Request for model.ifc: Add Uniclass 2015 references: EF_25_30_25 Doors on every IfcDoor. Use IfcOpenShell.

First a look at what the model holds.

```python
import ifcopenshell

model = ifcopenshell.open("model.ifc")
print(model.schema)
print("classifications:", [c.Name for c in model.by_type("IfcClassification")])
for ifc_class in ("IfcDoor", "IfcRoof", "IfcStair", "IfcWall", "IfcWindow"):
    print(ifc_class, len(model.by_type(ifc_class)))
```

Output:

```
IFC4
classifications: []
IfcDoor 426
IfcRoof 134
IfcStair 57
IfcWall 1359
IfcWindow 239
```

```python
import ifcopenshell
import ifcopenshell.api.classification

model = ifcopenshell.open("model.ifc")

system = ifcopenshell.api.classification.add_classification(model, classification="Uniclass 2015")

codes = {
    "IfcDoor": ("EF_25_30_25", "Doors"),
}
for ifc_class, (code, name) in codes.items():
    products = model.by_type(ifc_class)
    ifcopenshell.api.classification.add_reference(
        model, products=products, classification=system, identification=code, name=name
    )
    print(code, len(products))

model.write("model_edited.ifc")
```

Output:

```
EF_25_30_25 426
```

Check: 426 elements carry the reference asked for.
